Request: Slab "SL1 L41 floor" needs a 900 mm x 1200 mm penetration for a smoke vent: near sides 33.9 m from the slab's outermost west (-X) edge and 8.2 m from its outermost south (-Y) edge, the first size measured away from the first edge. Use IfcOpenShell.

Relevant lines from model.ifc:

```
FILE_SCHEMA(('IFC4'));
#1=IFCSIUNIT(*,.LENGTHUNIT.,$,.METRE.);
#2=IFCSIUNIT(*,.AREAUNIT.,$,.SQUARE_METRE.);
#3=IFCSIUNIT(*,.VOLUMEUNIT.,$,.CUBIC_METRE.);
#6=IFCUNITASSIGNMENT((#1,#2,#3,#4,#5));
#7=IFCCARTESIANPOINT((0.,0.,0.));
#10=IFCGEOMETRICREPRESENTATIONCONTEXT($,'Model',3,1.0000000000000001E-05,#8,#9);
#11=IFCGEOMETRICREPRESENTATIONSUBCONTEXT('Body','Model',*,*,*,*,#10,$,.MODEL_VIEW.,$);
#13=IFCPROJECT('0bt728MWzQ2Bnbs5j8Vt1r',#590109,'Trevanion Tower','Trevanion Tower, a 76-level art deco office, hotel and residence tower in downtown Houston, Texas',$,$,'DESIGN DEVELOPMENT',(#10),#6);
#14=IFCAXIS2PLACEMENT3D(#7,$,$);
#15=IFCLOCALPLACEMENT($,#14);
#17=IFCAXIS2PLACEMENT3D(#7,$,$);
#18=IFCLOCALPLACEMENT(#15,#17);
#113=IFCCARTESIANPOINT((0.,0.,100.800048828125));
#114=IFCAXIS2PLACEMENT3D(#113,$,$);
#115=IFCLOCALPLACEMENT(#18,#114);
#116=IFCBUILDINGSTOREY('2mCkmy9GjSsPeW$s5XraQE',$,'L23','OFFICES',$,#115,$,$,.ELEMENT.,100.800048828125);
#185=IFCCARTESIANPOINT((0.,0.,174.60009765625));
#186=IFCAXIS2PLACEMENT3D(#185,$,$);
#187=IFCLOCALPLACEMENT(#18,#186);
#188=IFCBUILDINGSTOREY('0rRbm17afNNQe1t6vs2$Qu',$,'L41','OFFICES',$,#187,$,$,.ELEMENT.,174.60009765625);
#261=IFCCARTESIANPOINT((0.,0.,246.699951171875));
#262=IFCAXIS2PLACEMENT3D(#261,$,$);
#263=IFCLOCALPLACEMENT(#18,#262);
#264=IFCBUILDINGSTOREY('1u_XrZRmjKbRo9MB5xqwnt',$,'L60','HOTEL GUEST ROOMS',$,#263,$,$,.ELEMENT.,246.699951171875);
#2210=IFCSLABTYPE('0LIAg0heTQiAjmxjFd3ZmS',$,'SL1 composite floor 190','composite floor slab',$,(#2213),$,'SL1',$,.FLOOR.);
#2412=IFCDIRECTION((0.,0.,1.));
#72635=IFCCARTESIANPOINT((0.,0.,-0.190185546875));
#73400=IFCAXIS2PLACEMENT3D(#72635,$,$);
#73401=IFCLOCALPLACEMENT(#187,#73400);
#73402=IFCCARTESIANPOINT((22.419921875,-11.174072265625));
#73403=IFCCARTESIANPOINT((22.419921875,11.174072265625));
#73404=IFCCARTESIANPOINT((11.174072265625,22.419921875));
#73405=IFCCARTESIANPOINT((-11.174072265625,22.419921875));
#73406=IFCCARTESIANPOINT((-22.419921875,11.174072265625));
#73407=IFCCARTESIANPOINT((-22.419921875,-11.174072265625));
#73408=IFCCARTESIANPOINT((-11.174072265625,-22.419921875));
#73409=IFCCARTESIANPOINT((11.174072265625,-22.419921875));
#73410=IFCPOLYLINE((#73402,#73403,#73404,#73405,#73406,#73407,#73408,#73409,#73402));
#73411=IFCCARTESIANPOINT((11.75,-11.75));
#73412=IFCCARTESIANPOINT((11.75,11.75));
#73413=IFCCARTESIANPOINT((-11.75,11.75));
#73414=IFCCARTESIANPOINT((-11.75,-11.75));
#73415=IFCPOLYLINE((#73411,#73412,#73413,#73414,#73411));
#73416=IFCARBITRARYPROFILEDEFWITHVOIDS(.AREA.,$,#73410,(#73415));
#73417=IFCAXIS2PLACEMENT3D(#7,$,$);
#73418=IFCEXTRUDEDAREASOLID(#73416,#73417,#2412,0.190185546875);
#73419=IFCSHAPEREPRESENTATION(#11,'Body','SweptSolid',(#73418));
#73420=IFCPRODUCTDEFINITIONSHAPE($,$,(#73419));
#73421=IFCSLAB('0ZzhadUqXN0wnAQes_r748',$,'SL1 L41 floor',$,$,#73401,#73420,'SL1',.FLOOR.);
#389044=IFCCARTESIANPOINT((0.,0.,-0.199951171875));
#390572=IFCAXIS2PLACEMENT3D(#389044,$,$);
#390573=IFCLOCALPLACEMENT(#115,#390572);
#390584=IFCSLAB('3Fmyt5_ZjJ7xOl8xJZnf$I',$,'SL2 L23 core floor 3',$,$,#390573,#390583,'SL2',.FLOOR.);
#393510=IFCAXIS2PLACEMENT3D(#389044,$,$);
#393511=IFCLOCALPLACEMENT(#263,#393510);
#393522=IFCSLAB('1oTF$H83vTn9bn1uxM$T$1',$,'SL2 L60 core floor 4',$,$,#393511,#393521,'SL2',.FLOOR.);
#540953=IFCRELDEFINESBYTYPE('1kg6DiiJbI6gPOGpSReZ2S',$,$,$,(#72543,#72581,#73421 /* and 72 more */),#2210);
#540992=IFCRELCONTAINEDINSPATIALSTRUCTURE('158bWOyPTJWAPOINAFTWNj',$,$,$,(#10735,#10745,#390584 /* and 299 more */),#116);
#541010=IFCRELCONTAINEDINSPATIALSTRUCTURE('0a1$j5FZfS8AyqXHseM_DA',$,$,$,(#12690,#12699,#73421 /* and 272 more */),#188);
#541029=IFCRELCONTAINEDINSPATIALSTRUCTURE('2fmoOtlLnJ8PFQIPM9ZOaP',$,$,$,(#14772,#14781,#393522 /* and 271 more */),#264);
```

```python
import numpy as np
import ifcopenshell
import ifcopenshell.api.feature
import ifcopenshell.api.geometry
import ifcopenshell.api.root
import ifcopenshell.geom
import ifcopenshell.util.placement
import ifcopenshell.util.representation
import ifcopenshell.util.shape
import ifcopenshell.util.unit

model = ifcopenshell.open("model.ifc")
unit_scale = ifcopenshell.util.unit.calculate_unit_scale(model)
settings = ifcopenshell.geom.settings()


def volume(element):
    """Net volume in cubic metres, openings subtracted."""
    shape = ifcopenshell.geom.create_shape(settings, element)
    return ifcopenshell.util.shape.get_volume(shape.geometry)


slab = model.by_guid("0ZzhadUqXN0wnAQes_r748")
before = volume(slab)

# Extent in the slab's own axes, in metres. The edges named are its -X and -Y sides.
slab_shape = ifcopenshell.geom.create_shape(settings, slab)
vertices = ifcopenshell.util.shape.get_vertices(slab_shape.geometry)
x_min, y_min, bottom = vertices.min(axis=0)
top = vertices[:, 2].max()

opening = ifcopenshell.api.root.create_entity(model, ifc_class="IfcOpeningElement", name="Smoke vent opening", predefined_type="OPENING")
context = ifcopenshell.util.representation.get_context(model, "Model", "Body", "MODEL_VIEW")
width, depth = 0.9, 1.2
outline = [(0.0, 0.0), (width, 0.0), (width, depth), (0.0, depth), (0.0, 0.0)]
# Overshoot both faces by 50 mm so the cut is clean.
shape = ifcopenshell.api.geometry.add_slab_representation(
    model, context=context, depth=top - bottom + 0.1, polyline=outline
)
ifcopenshell.api.geometry.assign_representation(model, product=opening, representation=shape)

matrix = ifcopenshell.util.placement.get_local_placement(slab.ObjectPlacement)
matrix[:, 3] = matrix @ np.append(np.array([x_min + 33.9, y_min + 8.2, bottom - 0.05]) / unit_scale, 1.0)
ifcopenshell.api.geometry.edit_object_placement(model, product=opening, matrix=matrix, is_si=False)
ifcopenshell.api.feature.add_feature(model, feature=opening, element=slab)

after = volume(slab)

print(f"slab volume {before:.3f} -> {after:.3f} m3")

model.write("model_rev.ifc")
```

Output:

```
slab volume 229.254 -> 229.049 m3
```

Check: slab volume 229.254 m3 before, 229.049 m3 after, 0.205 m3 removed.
